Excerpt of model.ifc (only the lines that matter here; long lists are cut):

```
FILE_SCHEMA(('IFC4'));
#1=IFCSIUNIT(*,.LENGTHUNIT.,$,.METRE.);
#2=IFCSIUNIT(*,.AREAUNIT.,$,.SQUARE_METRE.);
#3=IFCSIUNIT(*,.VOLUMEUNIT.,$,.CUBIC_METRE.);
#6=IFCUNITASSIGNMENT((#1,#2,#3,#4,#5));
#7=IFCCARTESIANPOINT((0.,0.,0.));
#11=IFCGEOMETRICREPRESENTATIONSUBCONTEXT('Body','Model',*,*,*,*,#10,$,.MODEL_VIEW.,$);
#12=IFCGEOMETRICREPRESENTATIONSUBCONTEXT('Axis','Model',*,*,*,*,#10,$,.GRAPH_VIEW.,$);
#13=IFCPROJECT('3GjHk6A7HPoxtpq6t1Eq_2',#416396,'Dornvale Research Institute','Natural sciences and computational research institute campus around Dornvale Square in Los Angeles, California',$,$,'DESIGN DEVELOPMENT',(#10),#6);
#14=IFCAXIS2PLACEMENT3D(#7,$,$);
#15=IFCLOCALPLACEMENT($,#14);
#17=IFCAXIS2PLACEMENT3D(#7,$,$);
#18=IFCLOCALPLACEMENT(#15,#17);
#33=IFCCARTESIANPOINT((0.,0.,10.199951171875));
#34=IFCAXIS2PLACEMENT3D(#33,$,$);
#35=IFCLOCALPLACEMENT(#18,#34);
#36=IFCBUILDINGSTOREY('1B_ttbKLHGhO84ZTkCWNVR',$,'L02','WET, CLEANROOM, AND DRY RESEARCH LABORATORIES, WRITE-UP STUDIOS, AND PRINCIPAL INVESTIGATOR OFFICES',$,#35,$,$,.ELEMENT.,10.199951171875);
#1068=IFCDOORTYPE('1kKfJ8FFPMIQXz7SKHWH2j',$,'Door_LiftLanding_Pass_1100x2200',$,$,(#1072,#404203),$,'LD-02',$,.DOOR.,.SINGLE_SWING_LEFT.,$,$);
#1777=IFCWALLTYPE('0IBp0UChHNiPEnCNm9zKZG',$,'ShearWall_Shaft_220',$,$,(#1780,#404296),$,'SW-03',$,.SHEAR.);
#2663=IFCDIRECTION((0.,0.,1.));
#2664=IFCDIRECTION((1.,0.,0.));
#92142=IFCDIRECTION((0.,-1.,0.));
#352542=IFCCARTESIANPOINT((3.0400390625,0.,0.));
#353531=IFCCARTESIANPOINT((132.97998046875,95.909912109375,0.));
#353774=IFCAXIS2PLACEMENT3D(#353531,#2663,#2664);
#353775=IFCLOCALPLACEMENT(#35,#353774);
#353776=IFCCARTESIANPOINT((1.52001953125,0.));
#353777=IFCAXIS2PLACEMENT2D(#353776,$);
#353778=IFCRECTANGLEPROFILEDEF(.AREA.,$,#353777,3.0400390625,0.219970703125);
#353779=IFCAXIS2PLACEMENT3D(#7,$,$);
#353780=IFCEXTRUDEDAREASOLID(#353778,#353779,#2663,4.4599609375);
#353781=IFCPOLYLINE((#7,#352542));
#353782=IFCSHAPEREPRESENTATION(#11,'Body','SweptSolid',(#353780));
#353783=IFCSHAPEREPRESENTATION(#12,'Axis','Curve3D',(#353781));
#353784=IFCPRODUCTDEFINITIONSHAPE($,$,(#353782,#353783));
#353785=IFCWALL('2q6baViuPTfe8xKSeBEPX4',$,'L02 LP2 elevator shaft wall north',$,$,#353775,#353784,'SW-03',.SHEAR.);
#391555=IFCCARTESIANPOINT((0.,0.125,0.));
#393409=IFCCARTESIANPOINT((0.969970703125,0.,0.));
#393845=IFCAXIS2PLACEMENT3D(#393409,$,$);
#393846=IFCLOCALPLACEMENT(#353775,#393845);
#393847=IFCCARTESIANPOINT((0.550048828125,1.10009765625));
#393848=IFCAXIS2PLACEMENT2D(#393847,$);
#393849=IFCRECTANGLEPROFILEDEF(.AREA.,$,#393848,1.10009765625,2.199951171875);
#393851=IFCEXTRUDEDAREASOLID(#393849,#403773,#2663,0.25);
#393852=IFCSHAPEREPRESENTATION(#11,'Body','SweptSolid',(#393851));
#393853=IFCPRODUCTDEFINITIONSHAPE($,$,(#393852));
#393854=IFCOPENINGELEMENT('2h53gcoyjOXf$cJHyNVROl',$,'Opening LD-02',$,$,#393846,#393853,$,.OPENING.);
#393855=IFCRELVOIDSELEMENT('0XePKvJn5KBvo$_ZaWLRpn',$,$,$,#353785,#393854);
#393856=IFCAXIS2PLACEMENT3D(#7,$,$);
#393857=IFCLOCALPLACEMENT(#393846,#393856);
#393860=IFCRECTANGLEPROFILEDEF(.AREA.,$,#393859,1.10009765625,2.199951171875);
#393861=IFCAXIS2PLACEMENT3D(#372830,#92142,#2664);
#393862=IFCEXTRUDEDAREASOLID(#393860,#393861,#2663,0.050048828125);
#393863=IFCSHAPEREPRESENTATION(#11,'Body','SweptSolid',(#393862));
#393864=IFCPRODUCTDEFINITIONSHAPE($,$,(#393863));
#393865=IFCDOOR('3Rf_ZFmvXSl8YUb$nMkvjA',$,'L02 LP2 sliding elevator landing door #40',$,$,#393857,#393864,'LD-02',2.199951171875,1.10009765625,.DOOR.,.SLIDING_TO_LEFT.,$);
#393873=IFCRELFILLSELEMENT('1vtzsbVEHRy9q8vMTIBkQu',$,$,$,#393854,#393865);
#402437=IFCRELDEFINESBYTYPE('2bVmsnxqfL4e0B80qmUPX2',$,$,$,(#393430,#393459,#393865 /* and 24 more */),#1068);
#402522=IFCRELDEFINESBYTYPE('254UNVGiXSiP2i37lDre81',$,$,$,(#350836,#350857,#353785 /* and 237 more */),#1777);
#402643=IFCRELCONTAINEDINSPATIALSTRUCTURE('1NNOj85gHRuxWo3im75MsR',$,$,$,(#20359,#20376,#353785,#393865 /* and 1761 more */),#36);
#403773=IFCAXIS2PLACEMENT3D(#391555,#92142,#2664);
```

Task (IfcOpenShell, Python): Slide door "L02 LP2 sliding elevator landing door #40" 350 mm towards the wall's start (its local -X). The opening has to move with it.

```python
import ifcopenshell
import ifcopenshell.api.geometry
import ifcopenshell.util.placement

model = ifcopenshell.open("model.ifc")

door = model.by_guid("3Rf_ZFmvXSl8YUb$nMkvjA")
opening = door.FillsVoids[0].RelatingOpeningElement
wall = opening.VoidsElements[0].RelatingBuildingElement

wall_matrix = ifcopenshell.util.placement.get_local_placement(wall.ObjectPlacement)
shift = wall_matrix[:3, 0] * -0.35
before = ifcopenshell.util.placement.get_local_placement(door.ObjectPlacement)[:3, 3].copy()

# The door is placed relative to its opening, so it follows when the opening moves.
matrix = ifcopenshell.util.placement.get_local_placement(opening.ObjectPlacement)
matrix[:3, 3] += shift
ifcopenshell.api.geometry.edit_object_placement(
    model, product=opening, matrix=matrix, is_si=False, should_transform_children=True
)

after = ifcopenshell.util.placement.get_local_placement(door.ObjectPlacement)[:3, 3]
print("door moved by", (after - before).round(3) + 0.0)

model.write("model_edited.ifc")
```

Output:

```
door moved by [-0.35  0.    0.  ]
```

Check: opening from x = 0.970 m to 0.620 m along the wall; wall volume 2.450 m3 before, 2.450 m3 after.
